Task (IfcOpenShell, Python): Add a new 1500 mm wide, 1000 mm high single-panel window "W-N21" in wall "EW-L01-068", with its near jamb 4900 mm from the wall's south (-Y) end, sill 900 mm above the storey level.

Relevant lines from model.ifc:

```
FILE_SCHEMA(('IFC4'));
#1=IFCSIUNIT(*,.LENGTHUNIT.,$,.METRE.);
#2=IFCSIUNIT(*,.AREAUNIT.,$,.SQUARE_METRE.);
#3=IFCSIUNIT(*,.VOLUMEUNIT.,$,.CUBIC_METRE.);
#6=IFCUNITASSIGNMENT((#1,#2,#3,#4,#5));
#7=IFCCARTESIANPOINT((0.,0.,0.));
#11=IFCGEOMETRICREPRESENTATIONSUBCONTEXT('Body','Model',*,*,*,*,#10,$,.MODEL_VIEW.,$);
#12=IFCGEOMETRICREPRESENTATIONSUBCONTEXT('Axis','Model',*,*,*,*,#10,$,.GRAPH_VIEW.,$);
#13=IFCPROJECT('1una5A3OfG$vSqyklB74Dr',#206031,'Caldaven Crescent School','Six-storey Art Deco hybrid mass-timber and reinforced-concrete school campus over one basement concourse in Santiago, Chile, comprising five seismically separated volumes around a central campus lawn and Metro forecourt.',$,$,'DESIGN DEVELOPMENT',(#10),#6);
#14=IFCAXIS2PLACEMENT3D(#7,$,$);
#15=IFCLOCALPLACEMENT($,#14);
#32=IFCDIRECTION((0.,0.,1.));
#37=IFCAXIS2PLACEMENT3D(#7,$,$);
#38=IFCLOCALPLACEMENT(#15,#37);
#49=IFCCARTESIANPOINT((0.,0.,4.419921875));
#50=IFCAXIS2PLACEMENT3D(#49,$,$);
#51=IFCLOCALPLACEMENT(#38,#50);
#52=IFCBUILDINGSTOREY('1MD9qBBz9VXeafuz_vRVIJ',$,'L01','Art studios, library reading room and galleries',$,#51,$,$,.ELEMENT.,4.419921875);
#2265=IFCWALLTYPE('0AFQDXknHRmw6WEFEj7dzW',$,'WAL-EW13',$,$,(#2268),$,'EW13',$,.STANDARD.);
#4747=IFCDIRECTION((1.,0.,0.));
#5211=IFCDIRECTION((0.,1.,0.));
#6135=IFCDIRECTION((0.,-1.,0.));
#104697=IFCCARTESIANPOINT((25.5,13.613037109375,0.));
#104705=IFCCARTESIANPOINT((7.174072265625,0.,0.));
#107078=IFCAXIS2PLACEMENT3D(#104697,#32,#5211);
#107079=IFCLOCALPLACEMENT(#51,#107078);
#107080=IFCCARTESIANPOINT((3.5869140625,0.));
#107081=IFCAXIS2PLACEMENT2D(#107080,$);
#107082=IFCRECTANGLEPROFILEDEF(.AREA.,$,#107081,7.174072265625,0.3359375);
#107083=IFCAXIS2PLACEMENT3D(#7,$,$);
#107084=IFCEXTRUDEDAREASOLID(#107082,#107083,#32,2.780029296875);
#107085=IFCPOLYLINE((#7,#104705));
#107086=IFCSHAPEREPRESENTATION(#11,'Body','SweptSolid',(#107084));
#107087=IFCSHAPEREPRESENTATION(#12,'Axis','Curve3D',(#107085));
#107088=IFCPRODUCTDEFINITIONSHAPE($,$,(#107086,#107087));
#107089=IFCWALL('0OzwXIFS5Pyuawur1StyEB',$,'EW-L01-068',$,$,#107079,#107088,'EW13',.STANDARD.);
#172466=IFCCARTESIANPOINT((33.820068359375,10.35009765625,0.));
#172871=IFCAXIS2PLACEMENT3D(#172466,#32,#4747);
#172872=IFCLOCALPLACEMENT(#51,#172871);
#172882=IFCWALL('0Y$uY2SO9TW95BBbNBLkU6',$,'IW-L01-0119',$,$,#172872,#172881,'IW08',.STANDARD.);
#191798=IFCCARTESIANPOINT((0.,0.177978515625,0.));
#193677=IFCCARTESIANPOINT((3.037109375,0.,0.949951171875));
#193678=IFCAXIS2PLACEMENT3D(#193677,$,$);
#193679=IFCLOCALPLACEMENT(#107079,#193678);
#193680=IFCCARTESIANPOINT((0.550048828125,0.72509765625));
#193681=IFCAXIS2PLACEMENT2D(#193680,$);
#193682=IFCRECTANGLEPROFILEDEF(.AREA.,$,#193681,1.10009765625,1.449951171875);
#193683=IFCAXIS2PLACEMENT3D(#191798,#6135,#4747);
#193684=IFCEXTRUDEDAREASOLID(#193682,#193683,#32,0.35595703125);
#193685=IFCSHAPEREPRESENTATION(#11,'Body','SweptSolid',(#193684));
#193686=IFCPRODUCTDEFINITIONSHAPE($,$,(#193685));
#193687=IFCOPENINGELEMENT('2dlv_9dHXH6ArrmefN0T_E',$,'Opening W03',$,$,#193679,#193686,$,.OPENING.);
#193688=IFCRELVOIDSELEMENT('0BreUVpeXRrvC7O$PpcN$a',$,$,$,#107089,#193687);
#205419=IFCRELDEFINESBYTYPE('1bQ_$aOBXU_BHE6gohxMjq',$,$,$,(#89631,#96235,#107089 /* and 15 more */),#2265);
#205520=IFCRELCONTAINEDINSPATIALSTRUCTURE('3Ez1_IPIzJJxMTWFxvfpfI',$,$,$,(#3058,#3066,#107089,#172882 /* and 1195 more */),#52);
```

```python
import numpy as np
import ifcopenshell
import ifcopenshell.api.feature
import ifcopenshell.api.geometry
import ifcopenshell.api.root
import ifcopenshell.api.spatial
import ifcopenshell.geom
import ifcopenshell.util.element
import ifcopenshell.util.placement
import ifcopenshell.util.representation
import ifcopenshell.util.shape
import ifcopenshell.util.unit

model = ifcopenshell.open("model.ifc")
unit_scale = ifcopenshell.util.unit.calculate_unit_scale(model)
settings = ifcopenshell.geom.settings()


def volume(element):
    """Net volume in cubic metres, openings subtracted."""
    shape = ifcopenshell.geom.create_shape(settings, element)
    return ifcopenshell.util.shape.get_volume(shape.geometry)


wall = model.by_id(107089)
storey = ifcopenshell.util.element.get_container(wall, ifc_class="IfcBuildingStorey")
context = ifcopenshell.util.representation.get_context(model, "Model", "Body", "MODEL_VIEW")
before = volume(wall)

width, height, from_end, sill = 1.5, 1, 4.9, 0.9  # metres

# The wall runs along its own X axis, and the end named is its -X end.
wall_shape = ifcopenshell.geom.create_shape(settings, wall)
x, y, z = ifcopenshell.util.shape.get_vertices(wall_shape.geometry).T
start = x.min() + from_end
face, thickness = float(y.min()), float(y.max() - y.min())
wall_matrix = ifcopenshell.util.placement.get_local_placement(wall.ObjectPlacement)
level = ifcopenshell.util.placement.get_local_placement(storey.ObjectPlacement)[2, 3]


def in_wall(x, y):
    """Placement at x, y metres in the wall's axes, at sill height."""
    matrix = wall_matrix.copy()
    matrix[:, 3] = wall_matrix @ np.array([x / unit_scale, y / unit_scale, 0.0, 1.0])
    matrix[2, 3] = level + sill / unit_scale
    return matrix


# Opening: a box that overshoots both wall faces by 50 mm.
opening = ifcopenshell.api.root.create_entity(model, ifc_class="IfcOpeningElement", predefined_type="OPENING")
box = ifcopenshell.api.geometry.add_wall_representation(
    model, context=context, length=width, height=height, thickness=thickness + 0.1
)
ifcopenshell.api.geometry.assign_representation(model, product=opening, representation=box)
ifcopenshell.api.geometry.edit_object_placement(model, product=opening, matrix=in_wall(start, face - 0.05), is_si=False)
ifcopenshell.api.feature.add_feature(model, feature=opening, element=wall)

window = ifcopenshell.api.root.create_entity(model, ifc_class="IfcWindow", name="W-N21", predefined_type="WINDOW")
window.OverallWidth, window.OverallHeight = width / unit_scale, height / unit_scale
window.PartitioningType = "SINGLE_PANEL"
body = ifcopenshell.api.geometry.add_window_representation(
    model,
    context=context,
    overall_width=window.OverallWidth,
    overall_height=window.OverallHeight,
    partition_type="SINGLE_PANEL",
)
ifcopenshell.api.geometry.assign_representation(model, product=window, representation=body)
ifcopenshell.api.spatial.assign_container(model, products=[window], relating_structure=storey)
ifcopenshell.api.feature.add_filling(model, opening=opening, element=window)

# Centre the window in the wall's thickness.
ifcopenshell.api.geometry.edit_object_placement(model, product=window, matrix=in_wall(start, face), is_si=False)
window_shape = ifcopenshell.geom.create_shape(settings, window)
depth = ifcopenshell.util.shape.get_vertices(window_shape.geometry)[:, 1]
offset = face + thickness / 2 - (depth.min() + depth.max()) / 2
ifcopenshell.api.geometry.edit_object_placement(model, product=window, matrix=in_wall(start, offset), is_si=False)

after = volume(wall)

print(f"wall volume {before:.3f} -> {after:.3f} m3")

model.write("model_v2.ifc")
```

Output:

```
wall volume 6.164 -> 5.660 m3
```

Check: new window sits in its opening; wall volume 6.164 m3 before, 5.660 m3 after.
